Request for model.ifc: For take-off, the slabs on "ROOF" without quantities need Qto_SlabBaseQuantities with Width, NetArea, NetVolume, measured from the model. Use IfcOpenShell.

First a look at what the model holds.

```python
import ifcopenshell
import ifcopenshell.util.element
import ifcopenshell.util.unit

model = ifcopenshell.open("model.ifc")
print(model.schema)
for unit_type in ("LENGTHUNIT", "AREAUNIT", "VOLUMEUNIT"):
    print(unit_type, ifcopenshell.util.unit.calculate_unit_scale(model, unit_type))
storey = next(s for s in model.by_type("IfcBuildingStorey") if s.Name == "ROOF")
slabs = [e for e in ifcopenshell.util.element.get_decomposition(storey) if e.is_a("IfcSlab")]
for e in sorted(slabs, key=lambda e: e.id()):
    print(e.id(), e.is_a(), e.Name, list(ifcopenshell.util.element.get_psets(e, qtos_only=True)), sep=" | ")
```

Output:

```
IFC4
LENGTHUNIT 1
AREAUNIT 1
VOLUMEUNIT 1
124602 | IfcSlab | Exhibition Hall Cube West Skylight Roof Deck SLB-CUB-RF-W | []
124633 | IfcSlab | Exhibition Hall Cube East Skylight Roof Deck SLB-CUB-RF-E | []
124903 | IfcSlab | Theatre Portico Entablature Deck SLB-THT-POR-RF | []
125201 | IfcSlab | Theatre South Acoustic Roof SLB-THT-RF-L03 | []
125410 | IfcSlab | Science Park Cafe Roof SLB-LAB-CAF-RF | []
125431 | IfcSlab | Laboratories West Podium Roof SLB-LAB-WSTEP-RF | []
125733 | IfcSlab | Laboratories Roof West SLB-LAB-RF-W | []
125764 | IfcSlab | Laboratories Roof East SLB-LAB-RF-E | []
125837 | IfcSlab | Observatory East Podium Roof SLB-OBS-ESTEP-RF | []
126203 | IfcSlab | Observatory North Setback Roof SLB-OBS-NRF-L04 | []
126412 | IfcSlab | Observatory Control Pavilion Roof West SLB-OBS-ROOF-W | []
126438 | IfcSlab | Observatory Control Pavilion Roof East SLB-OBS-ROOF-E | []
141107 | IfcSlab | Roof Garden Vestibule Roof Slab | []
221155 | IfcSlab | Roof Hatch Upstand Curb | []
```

```python
import ifcopenshell
import ifcopenshell.api.pset
import ifcopenshell.geom
import ifcopenshell.util.element
import ifcopenshell.util.shape
import ifcopenshell.util.unit

model = ifcopenshell.open("model.ifc")
unit_scale = ifcopenshell.util.unit.calculate_unit_scale(model)
area_scale = ifcopenshell.util.unit.calculate_unit_scale(model, "AREAUNIT")
volume_scale = ifcopenshell.util.unit.calculate_unit_scale(model, "VOLUMEUNIT")
settings = ifcopenshell.geom.settings()

storey = next(s for s in model.by_type("IfcBuildingStorey") if s.Name == "ROOF")
slabs = [e for e in ifcopenshell.util.element.get_decomposition(storey) if e.is_a("IfcSlab")]

for e in sorted(slabs, key=lambda e: e.id()):
    if ifcopenshell.util.element.get_psets(e, qtos_only=True, should_inherit=False):
        continue
    # Geometry comes back in metres, in the element's own axes.
    shape = ifcopenshell.geom.create_shape(settings, e)
    values = {
        "Width": ifcopenshell.util.shape.get_z(shape.geometry) / unit_scale,
        "NetArea": ifcopenshell.util.shape.get_footprint_area(shape.geometry) / area_scale,
        "NetVolume": ifcopenshell.util.shape.get_volume(shape.geometry) / volume_scale,
    }
    qto = ifcopenshell.api.pset.add_qto(model, product=e, name="Qto_SlabBaseQuantities")
    ifcopenshell.api.pset.edit_qto(model, qto=qto, properties=values)
    print(e.id(), {k: round(v, 3) for k, v in values.items()})

model.write("model-out.ifc")
```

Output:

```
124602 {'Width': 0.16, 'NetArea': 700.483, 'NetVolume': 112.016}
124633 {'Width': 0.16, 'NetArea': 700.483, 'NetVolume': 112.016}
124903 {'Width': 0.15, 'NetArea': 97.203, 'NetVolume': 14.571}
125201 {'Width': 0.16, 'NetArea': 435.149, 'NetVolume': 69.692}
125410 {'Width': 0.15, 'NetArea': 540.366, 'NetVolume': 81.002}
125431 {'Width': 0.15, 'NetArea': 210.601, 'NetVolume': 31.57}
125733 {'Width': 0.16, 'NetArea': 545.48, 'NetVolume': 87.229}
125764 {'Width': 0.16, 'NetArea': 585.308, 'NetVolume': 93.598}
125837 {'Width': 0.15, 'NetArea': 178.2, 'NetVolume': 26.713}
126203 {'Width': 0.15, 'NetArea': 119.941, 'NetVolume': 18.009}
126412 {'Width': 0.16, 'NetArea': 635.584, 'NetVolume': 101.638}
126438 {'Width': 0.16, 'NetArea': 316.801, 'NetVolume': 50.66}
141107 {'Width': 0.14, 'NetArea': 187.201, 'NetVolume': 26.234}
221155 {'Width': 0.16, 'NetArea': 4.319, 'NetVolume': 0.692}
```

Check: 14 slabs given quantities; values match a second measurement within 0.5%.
